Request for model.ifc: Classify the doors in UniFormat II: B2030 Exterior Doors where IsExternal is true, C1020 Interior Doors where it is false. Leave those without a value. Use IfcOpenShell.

First a look at what the model holds.

```python
import ifcopenshell
import ifcopenshell.util.element

model = ifcopenshell.open("model.ifc")
print(model.schema)
print("classifications:", [c.Name for c in model.by_type("IfcClassification")])
values = [ifcopenshell.util.element.get_pset(e, "Pset_DoorCommon", "IsExternal") for e in model.by_type("IfcDoor")]
for value in (True, False, None):
    print("IsExternal", value, values.count(value))
```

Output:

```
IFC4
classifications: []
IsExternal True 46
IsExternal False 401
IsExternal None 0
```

```python
import ifcopenshell
import ifcopenshell.api.classification
import ifcopenshell.util.element

model = ifcopenshell.open("model.ifc")

system = ifcopenshell.api.classification.add_classification(model, classification="UniFormat II")

doors = model.by_type("IfcDoor")
external = {e: ifcopenshell.util.element.get_pset(e, "Pset_DoorCommon", "IsExternal") for e in doors}
for flag, code, name in ((True, "B2030", "Exterior Doors"), (False, "C1020", "Interior Doors")):
    products = [e for e in doors if external[e] is flag]
    ifcopenshell.api.classification.add_reference(
        model, products=products, classification=system, identification=code, name=name
    )
    print(code, len(products))

model.write("model-out.ifc")
```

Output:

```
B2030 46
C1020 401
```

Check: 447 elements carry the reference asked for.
